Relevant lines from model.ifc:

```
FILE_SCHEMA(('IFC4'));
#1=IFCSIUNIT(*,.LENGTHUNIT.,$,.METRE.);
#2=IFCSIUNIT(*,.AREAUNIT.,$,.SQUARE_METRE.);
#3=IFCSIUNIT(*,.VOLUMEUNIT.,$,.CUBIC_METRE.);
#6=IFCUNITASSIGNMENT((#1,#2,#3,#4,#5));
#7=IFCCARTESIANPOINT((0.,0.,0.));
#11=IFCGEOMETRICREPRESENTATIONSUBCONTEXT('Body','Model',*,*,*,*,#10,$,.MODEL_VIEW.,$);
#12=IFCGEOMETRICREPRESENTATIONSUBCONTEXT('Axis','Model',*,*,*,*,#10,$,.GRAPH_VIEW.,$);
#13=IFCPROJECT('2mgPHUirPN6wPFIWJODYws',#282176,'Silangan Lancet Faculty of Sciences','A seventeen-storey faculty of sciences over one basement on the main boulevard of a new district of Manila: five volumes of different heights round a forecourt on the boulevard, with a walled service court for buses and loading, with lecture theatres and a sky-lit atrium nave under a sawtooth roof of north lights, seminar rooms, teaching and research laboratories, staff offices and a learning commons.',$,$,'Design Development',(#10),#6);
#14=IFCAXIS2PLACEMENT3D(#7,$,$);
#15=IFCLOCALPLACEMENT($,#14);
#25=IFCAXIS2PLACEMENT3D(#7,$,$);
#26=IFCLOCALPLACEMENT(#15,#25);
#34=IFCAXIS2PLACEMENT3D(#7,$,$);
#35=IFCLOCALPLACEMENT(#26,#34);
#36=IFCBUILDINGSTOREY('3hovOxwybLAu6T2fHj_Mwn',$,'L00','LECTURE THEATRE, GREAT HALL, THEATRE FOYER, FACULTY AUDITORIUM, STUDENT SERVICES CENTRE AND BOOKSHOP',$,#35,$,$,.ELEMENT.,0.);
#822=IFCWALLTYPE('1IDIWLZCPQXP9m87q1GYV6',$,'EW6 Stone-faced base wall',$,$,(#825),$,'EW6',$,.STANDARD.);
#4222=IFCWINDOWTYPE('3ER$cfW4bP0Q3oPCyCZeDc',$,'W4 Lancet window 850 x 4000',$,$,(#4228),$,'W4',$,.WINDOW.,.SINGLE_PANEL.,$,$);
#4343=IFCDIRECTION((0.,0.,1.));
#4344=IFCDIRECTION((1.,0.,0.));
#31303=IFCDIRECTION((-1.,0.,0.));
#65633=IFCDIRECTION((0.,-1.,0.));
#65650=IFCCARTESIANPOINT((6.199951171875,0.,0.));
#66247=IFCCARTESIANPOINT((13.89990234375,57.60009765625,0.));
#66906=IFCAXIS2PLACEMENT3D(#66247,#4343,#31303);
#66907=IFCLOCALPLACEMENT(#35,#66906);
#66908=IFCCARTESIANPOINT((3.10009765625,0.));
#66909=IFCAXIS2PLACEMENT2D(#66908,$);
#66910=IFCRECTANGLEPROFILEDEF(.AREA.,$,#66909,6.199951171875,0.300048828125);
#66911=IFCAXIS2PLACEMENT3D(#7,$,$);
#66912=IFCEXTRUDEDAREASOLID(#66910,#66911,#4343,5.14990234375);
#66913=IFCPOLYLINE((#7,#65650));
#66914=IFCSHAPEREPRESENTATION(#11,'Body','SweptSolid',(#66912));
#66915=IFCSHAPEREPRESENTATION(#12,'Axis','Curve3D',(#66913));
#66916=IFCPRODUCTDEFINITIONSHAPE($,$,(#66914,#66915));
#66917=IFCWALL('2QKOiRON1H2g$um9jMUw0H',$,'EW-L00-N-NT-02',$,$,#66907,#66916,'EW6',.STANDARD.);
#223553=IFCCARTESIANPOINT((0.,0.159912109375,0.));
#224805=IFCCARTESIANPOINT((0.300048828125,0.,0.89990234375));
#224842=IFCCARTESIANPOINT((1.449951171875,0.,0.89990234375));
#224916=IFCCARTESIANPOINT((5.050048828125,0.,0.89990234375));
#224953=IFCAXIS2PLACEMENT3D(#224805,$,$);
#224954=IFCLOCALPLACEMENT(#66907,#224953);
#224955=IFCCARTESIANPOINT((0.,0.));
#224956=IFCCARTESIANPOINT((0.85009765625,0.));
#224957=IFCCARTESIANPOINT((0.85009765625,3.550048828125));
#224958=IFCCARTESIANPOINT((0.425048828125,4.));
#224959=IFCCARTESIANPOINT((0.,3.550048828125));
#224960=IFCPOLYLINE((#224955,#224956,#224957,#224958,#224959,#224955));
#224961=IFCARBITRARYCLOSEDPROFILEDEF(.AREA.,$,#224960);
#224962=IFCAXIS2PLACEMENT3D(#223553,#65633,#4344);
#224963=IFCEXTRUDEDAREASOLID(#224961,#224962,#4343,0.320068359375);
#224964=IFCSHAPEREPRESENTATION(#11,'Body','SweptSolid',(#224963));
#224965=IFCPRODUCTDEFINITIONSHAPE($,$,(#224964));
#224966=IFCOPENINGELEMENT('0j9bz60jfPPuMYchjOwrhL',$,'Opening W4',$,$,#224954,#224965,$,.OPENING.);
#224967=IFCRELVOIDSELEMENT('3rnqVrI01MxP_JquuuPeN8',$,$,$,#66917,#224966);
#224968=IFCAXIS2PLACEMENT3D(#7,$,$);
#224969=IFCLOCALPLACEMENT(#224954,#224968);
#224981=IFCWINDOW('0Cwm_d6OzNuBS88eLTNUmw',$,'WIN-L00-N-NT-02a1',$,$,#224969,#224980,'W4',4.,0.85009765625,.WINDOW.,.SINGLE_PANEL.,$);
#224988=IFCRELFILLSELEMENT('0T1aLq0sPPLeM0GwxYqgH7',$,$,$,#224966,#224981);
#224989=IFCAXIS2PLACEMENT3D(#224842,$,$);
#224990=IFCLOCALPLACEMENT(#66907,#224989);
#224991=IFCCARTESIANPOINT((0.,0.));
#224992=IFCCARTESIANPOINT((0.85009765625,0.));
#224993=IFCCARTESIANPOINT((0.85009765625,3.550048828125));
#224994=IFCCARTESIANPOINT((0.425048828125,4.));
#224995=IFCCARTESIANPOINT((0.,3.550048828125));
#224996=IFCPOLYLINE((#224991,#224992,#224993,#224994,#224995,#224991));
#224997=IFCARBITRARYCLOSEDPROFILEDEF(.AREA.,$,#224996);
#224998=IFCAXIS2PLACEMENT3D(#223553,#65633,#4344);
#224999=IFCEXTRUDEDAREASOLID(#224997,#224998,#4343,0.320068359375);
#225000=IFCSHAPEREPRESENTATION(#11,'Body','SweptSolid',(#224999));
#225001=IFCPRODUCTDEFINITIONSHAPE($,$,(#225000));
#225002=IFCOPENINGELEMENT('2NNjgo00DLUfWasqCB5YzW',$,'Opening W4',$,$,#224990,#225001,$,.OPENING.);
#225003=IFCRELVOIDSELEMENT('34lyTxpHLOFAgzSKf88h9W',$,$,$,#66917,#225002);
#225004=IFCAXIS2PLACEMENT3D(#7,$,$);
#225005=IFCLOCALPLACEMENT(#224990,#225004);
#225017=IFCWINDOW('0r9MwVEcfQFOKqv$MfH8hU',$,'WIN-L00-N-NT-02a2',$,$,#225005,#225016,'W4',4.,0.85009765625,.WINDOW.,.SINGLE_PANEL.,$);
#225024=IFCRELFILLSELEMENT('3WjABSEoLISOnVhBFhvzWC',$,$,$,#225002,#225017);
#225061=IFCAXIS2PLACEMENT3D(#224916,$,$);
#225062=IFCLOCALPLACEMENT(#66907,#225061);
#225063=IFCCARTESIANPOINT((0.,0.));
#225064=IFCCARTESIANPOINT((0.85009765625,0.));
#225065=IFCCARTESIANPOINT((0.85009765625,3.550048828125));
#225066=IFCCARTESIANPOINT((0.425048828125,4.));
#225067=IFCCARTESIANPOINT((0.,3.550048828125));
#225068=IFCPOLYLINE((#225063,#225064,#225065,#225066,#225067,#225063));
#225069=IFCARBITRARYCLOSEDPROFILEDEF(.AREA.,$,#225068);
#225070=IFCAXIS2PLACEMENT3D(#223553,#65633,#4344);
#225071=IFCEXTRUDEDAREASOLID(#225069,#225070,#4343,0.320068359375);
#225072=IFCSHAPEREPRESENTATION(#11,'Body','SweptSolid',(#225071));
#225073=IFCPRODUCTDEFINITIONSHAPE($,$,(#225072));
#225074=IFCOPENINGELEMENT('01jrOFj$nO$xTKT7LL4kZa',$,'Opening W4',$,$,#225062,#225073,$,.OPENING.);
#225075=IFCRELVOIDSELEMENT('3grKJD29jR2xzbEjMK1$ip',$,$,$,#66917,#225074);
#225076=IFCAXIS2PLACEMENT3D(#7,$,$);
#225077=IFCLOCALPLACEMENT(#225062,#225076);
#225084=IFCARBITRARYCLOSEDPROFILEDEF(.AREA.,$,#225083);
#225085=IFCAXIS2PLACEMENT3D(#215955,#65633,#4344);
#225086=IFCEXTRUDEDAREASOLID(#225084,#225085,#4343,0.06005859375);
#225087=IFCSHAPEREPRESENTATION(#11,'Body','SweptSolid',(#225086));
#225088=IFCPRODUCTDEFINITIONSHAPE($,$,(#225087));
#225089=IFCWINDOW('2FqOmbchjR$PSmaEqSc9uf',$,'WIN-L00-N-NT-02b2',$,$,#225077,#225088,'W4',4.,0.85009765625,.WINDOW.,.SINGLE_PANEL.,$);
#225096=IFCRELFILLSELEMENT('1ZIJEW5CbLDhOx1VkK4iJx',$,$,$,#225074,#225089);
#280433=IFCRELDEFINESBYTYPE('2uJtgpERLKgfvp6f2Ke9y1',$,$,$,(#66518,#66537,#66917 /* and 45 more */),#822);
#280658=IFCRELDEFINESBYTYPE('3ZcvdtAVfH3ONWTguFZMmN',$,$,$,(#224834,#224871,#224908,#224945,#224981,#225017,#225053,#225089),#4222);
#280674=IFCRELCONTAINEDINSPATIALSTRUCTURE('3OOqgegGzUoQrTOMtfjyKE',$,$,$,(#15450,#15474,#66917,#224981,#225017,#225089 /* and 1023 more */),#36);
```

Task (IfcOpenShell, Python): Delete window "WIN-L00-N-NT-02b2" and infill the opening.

```python
import ifcopenshell
import ifcopenshell.api.feature
import ifcopenshell.api.root
import ifcopenshell.geom
import ifcopenshell.util.shape

model = ifcopenshell.open("model.ifc")
settings = ifcopenshell.geom.settings()


def volume(element):
    """Net volume in cubic metres, openings subtracted."""
    shape = ifcopenshell.geom.create_shape(settings, element)
    return ifcopenshell.util.shape.get_volume(shape.geometry)


window = model.by_guid("2FqOmbchjR$PSmaEqSc9uf")
opening = window.FillsVoids[0].RelatingOpeningElement
wall = opening.VoidsElements[0].RelatingBuildingElement
before = volume(wall)

ifcopenshell.api.root.remove_product(model, product=window)
ifcopenshell.api.feature.remove_feature(model, feature=opening)

after = volume(wall)

print(f"wall volume {before:.3f} -> {after:.3f} m3")

model.write("model_updated.ifc")
```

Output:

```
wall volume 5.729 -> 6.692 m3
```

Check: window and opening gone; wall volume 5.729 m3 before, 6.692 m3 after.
